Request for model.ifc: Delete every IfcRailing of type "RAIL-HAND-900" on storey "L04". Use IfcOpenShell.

First a look at what the model holds.

```python
import ifcopenshell
import ifcopenshell.util.element

model = ifcopenshell.open("model.ifc")
print(model.schema)
storey = next(s for s in model.by_type("IfcBuildingStorey") if s.Name == "L04")
railings = [e for e in ifcopenshell.util.element.get_decomposition(storey) if e.is_a("IfcRailing")]
seen = {}
for e in railings:
    element_type = ifcopenshell.util.element.get_type(e)
    name = element_type.Name if element_type not in (None, e) else None
    seen[name] = seen.get(name, 0) + 1
for name, count in sorted(seen.items(), key=str):
    print(count, "x", name)
```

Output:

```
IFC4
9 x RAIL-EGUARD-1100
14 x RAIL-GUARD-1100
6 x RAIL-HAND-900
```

```python
import ifcopenshell
import ifcopenshell.api.root
import ifcopenshell.util.element

model = ifcopenshell.open("model.ifc")

storey = next(s for s in model.by_type("IfcBuildingStorey") if s.Name == "L04")
railings = [e for e in ifcopenshell.util.element.get_decomposition(storey) if e.is_a("IfcRailing")]
targets = [e for e in railings if (t := ifcopenshell.util.element.get_type(e)) not in (None, e) and t.Name == "RAIL-HAND-900"]

for e in targets:
    ifcopenshell.api.root.remove_product(model, product=e)
print(len(targets), "removed")

model.write("model_rev.ifc")
```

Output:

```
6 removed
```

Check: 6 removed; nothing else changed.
